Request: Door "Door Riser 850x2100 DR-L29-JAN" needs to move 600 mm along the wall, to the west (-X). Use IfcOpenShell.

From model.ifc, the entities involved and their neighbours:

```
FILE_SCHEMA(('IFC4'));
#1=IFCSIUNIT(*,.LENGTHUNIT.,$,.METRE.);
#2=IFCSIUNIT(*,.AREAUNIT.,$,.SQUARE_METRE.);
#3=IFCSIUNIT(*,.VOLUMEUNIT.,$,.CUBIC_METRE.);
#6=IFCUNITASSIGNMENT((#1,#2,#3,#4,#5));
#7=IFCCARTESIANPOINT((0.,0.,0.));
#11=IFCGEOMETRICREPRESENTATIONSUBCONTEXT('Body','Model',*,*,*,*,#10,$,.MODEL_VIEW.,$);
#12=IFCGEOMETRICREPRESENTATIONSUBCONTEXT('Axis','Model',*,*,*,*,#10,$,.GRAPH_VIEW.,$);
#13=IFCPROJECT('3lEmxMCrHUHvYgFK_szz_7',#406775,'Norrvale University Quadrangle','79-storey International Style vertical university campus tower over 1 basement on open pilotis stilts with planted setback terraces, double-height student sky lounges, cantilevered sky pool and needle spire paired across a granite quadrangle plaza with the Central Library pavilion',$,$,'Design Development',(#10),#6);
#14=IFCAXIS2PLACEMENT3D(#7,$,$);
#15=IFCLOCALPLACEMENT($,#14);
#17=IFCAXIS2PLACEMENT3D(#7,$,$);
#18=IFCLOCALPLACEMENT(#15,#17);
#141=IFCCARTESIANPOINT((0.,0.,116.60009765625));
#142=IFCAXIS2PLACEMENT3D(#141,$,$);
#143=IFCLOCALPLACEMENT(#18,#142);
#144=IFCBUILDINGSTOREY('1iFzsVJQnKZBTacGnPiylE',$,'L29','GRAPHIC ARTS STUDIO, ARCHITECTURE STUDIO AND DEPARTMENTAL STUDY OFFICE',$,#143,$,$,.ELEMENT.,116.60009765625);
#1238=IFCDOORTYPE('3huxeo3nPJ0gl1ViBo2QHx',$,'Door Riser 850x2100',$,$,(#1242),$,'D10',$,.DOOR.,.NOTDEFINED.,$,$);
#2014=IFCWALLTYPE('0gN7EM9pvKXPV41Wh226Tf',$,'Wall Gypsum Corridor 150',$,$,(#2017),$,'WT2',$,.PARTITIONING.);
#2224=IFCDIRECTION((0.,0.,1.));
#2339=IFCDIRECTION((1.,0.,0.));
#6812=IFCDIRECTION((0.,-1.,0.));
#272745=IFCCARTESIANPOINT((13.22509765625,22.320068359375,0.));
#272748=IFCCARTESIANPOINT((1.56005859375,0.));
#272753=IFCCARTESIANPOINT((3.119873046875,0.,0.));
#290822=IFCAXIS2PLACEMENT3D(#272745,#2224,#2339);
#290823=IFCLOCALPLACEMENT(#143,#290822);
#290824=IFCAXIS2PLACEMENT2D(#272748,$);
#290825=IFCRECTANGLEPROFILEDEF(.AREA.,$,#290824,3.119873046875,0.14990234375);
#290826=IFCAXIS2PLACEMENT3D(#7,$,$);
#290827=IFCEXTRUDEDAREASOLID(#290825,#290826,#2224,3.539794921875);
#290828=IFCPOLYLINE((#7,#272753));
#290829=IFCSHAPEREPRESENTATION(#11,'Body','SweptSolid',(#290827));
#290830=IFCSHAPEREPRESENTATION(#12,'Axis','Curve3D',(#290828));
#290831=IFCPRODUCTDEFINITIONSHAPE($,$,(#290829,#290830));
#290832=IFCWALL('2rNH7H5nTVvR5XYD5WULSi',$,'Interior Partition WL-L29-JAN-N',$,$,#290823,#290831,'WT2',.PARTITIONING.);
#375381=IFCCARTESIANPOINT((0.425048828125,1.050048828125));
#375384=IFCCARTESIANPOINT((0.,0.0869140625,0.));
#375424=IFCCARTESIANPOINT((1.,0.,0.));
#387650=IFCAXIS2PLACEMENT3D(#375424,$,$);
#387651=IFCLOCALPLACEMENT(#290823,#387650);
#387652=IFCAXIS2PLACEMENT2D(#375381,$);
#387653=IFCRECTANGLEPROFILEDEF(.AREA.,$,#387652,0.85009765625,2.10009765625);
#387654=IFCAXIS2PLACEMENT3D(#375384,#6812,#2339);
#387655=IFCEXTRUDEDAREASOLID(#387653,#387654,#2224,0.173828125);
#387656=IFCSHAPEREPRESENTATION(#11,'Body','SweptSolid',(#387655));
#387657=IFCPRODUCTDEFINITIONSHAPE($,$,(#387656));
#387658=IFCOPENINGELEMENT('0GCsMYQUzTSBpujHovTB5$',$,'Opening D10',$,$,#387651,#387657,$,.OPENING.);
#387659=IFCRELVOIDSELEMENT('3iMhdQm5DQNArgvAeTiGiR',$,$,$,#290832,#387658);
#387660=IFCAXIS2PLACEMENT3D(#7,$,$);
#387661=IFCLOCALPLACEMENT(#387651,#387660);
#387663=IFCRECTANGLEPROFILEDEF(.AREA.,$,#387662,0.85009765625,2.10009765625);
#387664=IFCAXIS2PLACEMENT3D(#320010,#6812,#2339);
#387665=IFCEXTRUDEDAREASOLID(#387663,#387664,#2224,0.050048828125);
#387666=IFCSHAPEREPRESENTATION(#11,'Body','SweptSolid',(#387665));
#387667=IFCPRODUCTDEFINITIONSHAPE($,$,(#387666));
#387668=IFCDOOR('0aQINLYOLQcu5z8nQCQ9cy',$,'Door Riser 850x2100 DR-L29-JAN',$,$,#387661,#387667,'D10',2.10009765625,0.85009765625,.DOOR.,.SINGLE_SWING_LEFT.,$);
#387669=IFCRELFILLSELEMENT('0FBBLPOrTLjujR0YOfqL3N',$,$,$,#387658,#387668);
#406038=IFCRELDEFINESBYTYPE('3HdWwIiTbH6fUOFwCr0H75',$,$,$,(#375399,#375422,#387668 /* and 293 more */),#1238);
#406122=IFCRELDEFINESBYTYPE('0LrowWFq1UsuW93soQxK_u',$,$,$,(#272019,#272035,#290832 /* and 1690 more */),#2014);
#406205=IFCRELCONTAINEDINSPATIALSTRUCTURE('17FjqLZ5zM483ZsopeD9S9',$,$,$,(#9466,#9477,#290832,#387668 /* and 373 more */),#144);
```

```python
import ifcopenshell
import ifcopenshell.api.geometry
import ifcopenshell.util.placement

model = ifcopenshell.open("model.ifc")

door = model.by_guid("0aQINLYOLQcu5z8nQCQ9cy")
opening = door.FillsVoids[0].RelatingOpeningElement
wall = opening.VoidsElements[0].RelatingBuildingElement

wall_matrix = ifcopenshell.util.placement.get_local_placement(wall.ObjectPlacement)
shift = wall_matrix[:3, 0] * -0.6
before = ifcopenshell.util.placement.get_local_placement(door.ObjectPlacement)[:3, 3].copy()

# The door is placed relative to its opening, so it follows when the opening moves.
matrix = ifcopenshell.util.placement.get_local_placement(opening.ObjectPlacement)
matrix[:3, 3] += shift
ifcopenshell.api.geometry.edit_object_placement(
    model, product=opening, matrix=matrix, is_si=False, should_transform_children=True
)

after = ifcopenshell.util.placement.get_local_placement(door.ObjectPlacement)[:3, 3]
print("door moved by", (after - before).round(3) + 0.0)

model.write("model_v2.ifc")
```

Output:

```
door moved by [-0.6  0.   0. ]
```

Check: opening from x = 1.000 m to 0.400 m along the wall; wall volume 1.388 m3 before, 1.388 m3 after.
